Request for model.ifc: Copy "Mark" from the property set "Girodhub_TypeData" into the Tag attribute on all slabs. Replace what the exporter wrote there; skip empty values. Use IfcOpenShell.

First a look at what the model holds.

```python
import ifcopenshell
import ifcopenshell.util.element

model = ifcopenshell.open("model.ifc")
print(model.schema)
slabs = model.by_type("IfcSlab")
print(len(slabs), "slabs")
for e in slabs[:8]:
    source = ifcopenshell.util.element.get_pset(e, "Girodhub_TypeData", "Mark")
    target = e.Tag
    print(e.id(), repr(source), repr(target), sep=" | ")
```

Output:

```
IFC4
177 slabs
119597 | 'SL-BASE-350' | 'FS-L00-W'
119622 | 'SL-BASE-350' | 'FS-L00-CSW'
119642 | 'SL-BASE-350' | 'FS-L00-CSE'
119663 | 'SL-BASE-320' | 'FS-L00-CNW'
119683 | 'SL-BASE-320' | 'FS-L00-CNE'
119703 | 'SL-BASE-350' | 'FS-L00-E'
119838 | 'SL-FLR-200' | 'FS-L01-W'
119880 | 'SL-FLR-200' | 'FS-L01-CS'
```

```python
import ifcopenshell
import ifcopenshell.util.element

model = ifcopenshell.open("model.ifc")

count = 0
for e in model.by_type("IfcSlab"):
    value = ifcopenshell.util.element.get_pset(e, "Girodhub_TypeData", "Mark")
    current = e.Tag
    if not value or not value.strip() or current == value:
        continue
    e.Tag = value
    count += 1

print(count, "slabs updated")

model.write("model-out.ifc")
```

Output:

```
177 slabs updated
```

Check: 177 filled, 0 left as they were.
